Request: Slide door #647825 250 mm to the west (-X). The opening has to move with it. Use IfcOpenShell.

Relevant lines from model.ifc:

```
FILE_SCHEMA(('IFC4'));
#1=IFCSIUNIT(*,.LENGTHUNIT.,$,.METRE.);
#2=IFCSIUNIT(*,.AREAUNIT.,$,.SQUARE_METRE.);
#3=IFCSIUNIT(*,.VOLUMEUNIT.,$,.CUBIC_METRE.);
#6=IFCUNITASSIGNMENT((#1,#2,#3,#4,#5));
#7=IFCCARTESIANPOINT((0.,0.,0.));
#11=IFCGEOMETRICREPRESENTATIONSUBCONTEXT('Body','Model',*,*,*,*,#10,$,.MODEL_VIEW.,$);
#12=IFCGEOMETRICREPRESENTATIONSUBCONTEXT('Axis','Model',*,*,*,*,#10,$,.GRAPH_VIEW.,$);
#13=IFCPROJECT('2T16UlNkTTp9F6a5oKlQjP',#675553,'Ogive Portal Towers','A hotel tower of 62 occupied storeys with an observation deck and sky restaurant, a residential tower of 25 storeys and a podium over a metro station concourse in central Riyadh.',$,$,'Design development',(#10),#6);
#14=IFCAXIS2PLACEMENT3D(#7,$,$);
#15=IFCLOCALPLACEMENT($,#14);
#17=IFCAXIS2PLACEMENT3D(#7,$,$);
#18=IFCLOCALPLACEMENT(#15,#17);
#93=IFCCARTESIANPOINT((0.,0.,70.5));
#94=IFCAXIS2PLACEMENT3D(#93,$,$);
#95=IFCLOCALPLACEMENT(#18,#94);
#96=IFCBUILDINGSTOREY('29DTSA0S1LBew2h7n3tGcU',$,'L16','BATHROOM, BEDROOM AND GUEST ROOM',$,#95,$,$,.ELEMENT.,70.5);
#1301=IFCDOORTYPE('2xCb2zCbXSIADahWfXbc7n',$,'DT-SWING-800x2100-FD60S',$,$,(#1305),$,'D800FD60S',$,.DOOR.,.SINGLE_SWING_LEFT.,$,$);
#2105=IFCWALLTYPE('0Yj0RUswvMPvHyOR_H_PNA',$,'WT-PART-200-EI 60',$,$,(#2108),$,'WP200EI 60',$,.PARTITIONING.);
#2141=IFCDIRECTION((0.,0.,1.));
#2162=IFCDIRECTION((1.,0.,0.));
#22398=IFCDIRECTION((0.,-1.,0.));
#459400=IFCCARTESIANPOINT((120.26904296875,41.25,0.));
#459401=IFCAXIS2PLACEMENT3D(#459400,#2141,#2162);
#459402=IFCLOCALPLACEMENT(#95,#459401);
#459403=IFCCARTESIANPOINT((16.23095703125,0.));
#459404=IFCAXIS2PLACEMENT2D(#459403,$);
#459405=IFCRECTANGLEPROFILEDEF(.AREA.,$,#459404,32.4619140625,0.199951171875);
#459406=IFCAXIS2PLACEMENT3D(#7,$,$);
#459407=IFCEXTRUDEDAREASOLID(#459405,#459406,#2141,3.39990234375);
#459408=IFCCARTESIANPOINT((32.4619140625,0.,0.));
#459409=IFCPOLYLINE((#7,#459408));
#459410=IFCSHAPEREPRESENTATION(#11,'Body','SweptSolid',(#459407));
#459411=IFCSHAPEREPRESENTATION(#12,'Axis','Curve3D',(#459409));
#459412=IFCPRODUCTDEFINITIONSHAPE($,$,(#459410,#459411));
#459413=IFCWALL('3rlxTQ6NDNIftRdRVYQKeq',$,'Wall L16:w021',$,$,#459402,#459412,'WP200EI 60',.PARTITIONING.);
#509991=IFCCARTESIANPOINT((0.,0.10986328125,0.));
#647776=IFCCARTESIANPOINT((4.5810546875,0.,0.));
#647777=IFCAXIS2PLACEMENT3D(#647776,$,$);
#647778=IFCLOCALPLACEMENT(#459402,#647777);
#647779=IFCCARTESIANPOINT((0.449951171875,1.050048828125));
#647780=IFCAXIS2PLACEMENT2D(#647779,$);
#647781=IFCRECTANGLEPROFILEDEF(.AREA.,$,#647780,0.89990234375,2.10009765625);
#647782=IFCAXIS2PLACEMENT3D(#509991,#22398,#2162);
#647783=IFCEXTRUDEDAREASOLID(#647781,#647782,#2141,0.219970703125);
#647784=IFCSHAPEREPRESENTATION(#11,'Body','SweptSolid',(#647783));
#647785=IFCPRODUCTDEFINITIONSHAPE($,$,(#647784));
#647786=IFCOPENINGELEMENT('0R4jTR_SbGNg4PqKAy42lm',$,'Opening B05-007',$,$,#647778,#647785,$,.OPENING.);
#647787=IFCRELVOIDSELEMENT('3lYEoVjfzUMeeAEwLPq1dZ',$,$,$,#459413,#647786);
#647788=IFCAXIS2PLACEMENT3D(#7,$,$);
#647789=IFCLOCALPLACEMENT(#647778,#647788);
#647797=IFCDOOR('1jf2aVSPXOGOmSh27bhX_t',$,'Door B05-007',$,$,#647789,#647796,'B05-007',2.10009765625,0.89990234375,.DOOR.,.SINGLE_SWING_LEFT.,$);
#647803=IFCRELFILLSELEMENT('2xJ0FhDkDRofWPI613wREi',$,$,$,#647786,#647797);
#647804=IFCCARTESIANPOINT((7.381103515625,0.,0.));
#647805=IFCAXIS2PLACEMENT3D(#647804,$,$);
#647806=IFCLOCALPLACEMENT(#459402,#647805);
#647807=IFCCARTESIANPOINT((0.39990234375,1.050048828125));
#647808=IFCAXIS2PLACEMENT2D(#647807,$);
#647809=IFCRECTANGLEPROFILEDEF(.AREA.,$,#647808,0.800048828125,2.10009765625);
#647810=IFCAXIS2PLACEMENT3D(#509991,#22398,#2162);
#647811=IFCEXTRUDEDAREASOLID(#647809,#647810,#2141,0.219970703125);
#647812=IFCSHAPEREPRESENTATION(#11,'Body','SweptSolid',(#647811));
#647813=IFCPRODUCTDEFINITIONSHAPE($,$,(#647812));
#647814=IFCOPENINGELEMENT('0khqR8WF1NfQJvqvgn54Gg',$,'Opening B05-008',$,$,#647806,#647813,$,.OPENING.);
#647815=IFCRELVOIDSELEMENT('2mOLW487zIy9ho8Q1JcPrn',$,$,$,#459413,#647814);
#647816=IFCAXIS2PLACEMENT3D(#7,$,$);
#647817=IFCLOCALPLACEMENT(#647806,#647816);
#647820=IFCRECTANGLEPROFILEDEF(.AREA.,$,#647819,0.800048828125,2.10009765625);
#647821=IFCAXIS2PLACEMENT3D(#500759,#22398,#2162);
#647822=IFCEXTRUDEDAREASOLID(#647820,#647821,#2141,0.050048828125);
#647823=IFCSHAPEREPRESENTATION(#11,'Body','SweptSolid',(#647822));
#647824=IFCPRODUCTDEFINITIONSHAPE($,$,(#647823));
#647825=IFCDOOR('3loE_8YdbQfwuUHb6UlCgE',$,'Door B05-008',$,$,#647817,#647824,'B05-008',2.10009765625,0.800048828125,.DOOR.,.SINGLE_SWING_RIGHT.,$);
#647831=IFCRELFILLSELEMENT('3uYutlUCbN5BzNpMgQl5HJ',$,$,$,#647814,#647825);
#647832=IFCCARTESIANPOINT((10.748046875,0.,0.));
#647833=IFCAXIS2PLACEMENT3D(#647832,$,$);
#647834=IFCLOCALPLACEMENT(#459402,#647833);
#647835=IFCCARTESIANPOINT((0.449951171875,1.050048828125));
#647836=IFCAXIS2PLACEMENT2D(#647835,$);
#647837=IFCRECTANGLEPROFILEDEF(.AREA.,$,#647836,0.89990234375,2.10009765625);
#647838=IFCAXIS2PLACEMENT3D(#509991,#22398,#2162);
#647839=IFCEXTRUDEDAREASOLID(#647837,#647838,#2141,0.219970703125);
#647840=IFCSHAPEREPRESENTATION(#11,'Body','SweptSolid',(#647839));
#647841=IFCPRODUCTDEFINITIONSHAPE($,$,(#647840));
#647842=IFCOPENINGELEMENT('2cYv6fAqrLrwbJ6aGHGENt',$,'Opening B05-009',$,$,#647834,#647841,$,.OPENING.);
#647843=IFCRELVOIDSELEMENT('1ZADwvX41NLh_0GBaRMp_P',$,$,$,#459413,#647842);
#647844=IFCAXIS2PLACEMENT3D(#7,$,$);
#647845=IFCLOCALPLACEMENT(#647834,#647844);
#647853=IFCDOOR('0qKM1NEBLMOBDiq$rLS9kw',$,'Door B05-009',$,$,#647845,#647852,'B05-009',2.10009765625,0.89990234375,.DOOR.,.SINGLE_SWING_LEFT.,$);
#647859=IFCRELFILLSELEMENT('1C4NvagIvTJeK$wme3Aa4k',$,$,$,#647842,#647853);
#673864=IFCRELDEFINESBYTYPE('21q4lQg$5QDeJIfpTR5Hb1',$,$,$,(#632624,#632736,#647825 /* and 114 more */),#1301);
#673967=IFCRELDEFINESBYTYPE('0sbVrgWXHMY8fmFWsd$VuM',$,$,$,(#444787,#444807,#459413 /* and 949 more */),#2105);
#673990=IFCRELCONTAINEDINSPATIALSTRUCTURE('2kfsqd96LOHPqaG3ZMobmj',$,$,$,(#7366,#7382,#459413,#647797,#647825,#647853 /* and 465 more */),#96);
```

```python
import ifcopenshell
import ifcopenshell.api.geometry
import ifcopenshell.util.placement
import ifcopenshell.util.unit

model = ifcopenshell.open("model.ifc")
unit_scale = ifcopenshell.util.unit.calculate_unit_scale(model)

door = model.by_guid("3loE_8YdbQfwuUHb6UlCgE")
opening = door.FillsVoids[0].RelatingOpeningElement
wall = opening.VoidsElements[0].RelatingBuildingElement

wall_matrix = ifcopenshell.util.placement.get_local_placement(wall.ObjectPlacement)
shift = wall_matrix[:3, 0] * -0.25 / unit_scale
before = ifcopenshell.util.placement.get_local_placement(door.ObjectPlacement)[:3, 3].copy()

# The door is placed relative to its opening, so it follows when the opening moves.
matrix = ifcopenshell.util.placement.get_local_placement(opening.ObjectPlacement)
matrix[:3, 3] += shift
ifcopenshell.api.geometry.edit_object_placement(
    model, product=opening, matrix=matrix, is_si=False, should_transform_children=True
)

after = ifcopenshell.util.placement.get_local_placement(door.ObjectPlacement)[:3, 3]
print("door moved by", (after - before).round(3) + 0.0)

model.write("model_edited.ifc")
```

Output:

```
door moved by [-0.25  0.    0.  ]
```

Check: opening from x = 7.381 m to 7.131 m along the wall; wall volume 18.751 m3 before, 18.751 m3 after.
